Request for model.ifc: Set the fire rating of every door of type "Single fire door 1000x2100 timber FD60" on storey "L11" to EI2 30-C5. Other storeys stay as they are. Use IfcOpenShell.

First a look at what the model holds.

```python
import ifcopenshell
import ifcopenshell.util.element

model = ifcopenshell.open("model.ifc")
print(model.schema)
storey = next(s for s in model.by_type("IfcBuildingStorey") if s.Name == "L11")
doors = [e for e in ifcopenshell.util.element.get_decomposition(storey) if e.is_a("IfcDoor")]
seen = {}
for e in doors:
    element_type = ifcopenshell.util.element.get_type(e)
    key = (element_type.Name if element_type != e and element_type else None, ifcopenshell.util.element.get_pset(e, "Pset_DoorCommon", "FireRating"))
    seen[key] = seen.get(key, 0) + 1
for (name, value), count in sorted(seen.items(), key=str):
    print(count, "x", name, "|", value)
```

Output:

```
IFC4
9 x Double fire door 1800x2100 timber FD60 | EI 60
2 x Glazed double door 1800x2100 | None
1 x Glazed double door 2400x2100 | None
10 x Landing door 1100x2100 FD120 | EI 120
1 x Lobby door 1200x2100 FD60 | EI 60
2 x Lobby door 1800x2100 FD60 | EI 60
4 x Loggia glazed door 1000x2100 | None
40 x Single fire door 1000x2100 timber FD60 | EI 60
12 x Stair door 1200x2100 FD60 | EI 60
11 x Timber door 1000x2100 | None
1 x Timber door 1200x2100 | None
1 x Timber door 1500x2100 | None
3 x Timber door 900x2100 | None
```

```python
import ifcopenshell
import ifcopenshell.api.pset
import ifcopenshell.util.element

model = ifcopenshell.open("model.ifc")

storey = next(s for s in model.by_type("IfcBuildingStorey") if s.Name == "L11")
doors = [e for e in ifcopenshell.util.element.get_decomposition(storey) if e.is_a("IfcDoor")]

count = 0
for e in doors:
    element_type = ifcopenshell.util.element.get_type(e)
    if element_type in (None, e) or element_type.Name != "Single fire door 1000x2100 timber FD60":
        continue
    found = ifcopenshell.util.element.get_pset(e, "Pset_DoorCommon", should_inherit=False)
    if found:
        pset = model.by_id(found["id"])
        if len(ifcopenshell.util.element.get_elements_by_pset(pset)) > 1:
            pset = ifcopenshell.api.pset.unshare_pset(model, products=[e], pset=pset)[0]
    else:
        pset = ifcopenshell.api.pset.add_pset(model, product=e, name="Pset_DoorCommon")
    ifcopenshell.api.pset.edit_pset(model, pset=pset, properties={"FireRating": "EI2 30-C5"})
    count += 1

print(count, "doors updated")

model.write("model-out.ifc")
```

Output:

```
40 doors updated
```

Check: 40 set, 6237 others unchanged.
